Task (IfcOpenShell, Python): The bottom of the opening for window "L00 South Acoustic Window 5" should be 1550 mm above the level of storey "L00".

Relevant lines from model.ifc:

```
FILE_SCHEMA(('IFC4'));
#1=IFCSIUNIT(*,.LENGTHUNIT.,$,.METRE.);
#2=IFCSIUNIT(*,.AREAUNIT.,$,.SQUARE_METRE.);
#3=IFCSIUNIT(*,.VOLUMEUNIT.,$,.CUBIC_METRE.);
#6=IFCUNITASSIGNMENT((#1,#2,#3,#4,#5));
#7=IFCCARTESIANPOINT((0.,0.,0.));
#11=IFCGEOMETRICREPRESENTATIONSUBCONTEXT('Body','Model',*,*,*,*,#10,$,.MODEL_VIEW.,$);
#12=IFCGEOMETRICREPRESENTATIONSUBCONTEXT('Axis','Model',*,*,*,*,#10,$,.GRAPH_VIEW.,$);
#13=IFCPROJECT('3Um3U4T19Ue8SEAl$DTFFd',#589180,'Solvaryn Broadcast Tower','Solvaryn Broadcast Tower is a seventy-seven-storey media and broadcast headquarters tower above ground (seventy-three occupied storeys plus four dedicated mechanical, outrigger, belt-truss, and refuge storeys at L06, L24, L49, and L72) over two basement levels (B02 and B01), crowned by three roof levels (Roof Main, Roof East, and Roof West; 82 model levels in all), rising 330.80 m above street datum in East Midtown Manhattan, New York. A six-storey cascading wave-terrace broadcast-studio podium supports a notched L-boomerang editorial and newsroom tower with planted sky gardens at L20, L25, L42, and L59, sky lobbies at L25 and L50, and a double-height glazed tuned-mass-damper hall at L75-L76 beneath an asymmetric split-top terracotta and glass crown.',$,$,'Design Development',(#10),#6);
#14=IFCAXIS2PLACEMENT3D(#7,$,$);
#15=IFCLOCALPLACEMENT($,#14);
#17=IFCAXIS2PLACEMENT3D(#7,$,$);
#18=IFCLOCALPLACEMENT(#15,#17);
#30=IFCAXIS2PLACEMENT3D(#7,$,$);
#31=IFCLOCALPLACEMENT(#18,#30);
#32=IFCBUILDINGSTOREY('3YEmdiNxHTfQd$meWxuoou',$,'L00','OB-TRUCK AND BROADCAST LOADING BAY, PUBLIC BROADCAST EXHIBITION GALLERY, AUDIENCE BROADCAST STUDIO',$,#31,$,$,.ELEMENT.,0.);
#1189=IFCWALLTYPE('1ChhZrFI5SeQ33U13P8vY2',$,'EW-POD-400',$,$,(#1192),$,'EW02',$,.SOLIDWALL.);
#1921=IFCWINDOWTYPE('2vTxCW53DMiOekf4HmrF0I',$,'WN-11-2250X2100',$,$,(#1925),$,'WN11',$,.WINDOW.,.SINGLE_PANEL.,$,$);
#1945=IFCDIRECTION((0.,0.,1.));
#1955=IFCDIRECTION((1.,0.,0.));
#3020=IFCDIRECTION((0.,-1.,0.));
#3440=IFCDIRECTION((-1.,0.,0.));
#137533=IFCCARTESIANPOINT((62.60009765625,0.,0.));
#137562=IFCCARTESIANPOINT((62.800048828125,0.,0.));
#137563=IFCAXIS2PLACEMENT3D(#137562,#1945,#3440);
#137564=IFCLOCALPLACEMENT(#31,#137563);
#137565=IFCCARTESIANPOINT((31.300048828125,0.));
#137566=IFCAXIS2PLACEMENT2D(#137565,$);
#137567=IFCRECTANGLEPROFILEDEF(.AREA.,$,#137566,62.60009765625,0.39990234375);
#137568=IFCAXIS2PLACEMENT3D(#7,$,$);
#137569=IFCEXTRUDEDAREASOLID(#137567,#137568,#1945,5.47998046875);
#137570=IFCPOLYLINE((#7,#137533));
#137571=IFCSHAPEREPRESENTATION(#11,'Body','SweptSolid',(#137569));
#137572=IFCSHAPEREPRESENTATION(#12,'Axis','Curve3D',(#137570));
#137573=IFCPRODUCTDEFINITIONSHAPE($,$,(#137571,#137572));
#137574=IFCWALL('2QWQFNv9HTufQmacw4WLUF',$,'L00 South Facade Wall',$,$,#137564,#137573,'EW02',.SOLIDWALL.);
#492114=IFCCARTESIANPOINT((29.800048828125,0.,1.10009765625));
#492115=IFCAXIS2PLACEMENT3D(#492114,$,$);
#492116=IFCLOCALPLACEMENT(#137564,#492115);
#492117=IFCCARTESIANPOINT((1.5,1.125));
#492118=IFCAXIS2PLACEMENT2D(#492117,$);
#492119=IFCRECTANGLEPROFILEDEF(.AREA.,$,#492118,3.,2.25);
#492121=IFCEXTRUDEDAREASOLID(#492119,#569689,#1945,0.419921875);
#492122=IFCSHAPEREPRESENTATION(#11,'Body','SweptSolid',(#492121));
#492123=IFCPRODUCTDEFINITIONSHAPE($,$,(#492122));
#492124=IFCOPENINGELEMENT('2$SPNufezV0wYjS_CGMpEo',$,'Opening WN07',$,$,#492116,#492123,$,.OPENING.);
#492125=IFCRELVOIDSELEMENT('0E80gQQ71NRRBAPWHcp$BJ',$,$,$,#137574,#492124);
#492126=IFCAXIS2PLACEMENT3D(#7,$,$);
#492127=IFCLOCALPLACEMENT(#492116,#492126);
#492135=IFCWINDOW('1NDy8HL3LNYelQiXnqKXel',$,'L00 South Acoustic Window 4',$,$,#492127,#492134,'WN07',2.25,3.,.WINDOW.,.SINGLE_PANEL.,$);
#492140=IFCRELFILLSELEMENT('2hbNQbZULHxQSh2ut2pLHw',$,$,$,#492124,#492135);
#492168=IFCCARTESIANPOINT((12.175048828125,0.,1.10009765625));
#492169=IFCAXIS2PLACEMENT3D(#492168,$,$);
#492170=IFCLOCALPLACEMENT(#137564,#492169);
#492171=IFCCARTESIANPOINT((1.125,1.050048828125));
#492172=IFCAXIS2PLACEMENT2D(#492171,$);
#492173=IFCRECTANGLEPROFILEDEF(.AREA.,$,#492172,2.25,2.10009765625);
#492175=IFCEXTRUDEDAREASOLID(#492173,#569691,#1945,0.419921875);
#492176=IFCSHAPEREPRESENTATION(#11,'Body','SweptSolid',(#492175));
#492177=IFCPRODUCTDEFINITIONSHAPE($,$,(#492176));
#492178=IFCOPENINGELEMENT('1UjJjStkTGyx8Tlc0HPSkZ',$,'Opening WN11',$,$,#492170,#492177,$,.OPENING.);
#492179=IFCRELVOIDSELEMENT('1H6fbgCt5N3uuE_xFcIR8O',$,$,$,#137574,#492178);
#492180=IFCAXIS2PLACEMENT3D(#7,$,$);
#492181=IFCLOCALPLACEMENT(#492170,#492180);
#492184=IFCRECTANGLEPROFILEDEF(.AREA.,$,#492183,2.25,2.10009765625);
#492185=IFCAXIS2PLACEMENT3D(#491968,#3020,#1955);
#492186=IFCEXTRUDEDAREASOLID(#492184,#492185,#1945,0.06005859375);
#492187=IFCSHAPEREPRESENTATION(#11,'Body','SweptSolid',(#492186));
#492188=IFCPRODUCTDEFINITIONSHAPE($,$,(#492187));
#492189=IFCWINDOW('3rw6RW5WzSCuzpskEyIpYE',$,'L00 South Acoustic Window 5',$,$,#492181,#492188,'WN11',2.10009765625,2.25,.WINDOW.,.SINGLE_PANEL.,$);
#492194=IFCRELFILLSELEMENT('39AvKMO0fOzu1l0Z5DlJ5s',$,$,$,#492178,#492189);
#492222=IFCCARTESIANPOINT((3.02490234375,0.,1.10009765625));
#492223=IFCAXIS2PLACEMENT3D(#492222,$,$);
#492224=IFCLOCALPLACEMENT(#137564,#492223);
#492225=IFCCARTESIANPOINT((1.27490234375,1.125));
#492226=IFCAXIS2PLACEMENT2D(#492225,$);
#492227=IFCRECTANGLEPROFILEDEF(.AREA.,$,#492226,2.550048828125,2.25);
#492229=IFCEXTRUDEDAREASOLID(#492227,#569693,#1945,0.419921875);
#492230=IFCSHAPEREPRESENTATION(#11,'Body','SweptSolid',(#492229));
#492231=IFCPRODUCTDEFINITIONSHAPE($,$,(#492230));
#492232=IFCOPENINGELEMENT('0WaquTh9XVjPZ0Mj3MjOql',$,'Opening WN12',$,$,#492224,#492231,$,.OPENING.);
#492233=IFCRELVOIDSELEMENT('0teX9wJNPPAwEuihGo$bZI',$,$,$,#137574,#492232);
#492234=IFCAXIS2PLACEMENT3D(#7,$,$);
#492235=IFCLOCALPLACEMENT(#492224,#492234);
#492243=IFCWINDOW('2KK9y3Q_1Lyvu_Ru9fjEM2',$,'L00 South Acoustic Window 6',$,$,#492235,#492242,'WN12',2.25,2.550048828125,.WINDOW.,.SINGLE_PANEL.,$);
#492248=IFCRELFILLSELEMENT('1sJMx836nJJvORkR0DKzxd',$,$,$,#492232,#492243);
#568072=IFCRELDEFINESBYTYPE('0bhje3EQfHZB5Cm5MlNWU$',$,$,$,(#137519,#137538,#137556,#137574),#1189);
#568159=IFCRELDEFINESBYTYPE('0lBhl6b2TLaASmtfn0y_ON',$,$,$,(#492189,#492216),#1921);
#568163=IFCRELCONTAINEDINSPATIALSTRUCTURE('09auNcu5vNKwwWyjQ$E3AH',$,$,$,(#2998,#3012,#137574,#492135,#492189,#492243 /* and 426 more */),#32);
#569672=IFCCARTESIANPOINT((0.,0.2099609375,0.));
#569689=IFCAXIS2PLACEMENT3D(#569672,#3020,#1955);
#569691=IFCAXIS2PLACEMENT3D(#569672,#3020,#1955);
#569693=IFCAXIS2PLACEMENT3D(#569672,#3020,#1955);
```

```python
import numpy as np
import ifcopenshell
import ifcopenshell.api.geometry
import ifcopenshell.geom
import ifcopenshell.util.element
import ifcopenshell.util.placement
import ifcopenshell.util.shape
import ifcopenshell.util.unit

model = ifcopenshell.open("model.ifc")
unit_scale = ifcopenshell.util.unit.calculate_unit_scale(model)

window = model.by_guid("3rw6RW5WzSCuzpskEyIpYE")
opening = window.FillsVoids[0].RelatingOpeningElement
storey = ifcopenshell.util.element.get_container(window, ifc_class="IfcBuildingStorey")
level = ifcopenshell.util.placement.get_local_placement(storey.ObjectPlacement)[2, 3]

# The opening's origin need not be at the sill, so measure its lowest point.
shape = ifcopenshell.geom.create_shape(ifcopenshell.geom.settings(), opening)
bottom = ifcopenshell.util.shape.get_shape_bottom_elevation(shape, shape.geometry) / unit_scale
dz = level + 1.55 / unit_scale - bottom

shift = np.array([0.0, 0.0, dz])
# The window is placed relative to its opening, so it follows when the opening moves.
matrix = ifcopenshell.util.placement.get_local_placement(opening.ObjectPlacement)
matrix[:3, 3] += shift
ifcopenshell.api.geometry.edit_object_placement(
    model, product=opening, matrix=matrix, is_si=False, should_transform_children=True
)

print(f"moved by {dz * unit_scale:+.3f} m")

model.write("model_edited.ifc")
```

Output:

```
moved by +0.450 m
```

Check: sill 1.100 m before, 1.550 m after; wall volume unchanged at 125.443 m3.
